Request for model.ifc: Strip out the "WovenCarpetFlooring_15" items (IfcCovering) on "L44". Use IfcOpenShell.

First a look at what the model holds.

```python
import ifcopenshell
import ifcopenshell.util.element

model = ifcopenshell.open("model.ifc")
print(model.schema)
storey = next(s for s in model.by_type("IfcBuildingStorey") if s.Name == "L44")
coverings = [e for e in ifcopenshell.util.element.get_decomposition(storey) if e.is_a("IfcCovering")]
seen = {}
for e in coverings:
    element_type = ifcopenshell.util.element.get_type(e)
    name = element_type.Name if element_type not in (None, e) else None
    seen[name] = seen.get(name, 0) + 1
for name, count in sorted(seen.items(), key=str):
    print(count, "x", name)
```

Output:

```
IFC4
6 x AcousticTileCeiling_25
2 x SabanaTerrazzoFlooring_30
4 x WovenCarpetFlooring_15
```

```python
import ifcopenshell
import ifcopenshell.api.root
import ifcopenshell.util.element

model = ifcopenshell.open("model.ifc")

storey = next(s for s in model.by_type("IfcBuildingStorey") if s.Name == "L44")
coverings = [e for e in ifcopenshell.util.element.get_decomposition(storey) if e.is_a("IfcCovering")]
targets = [e for e in coverings if (t := ifcopenshell.util.element.get_type(e)) not in (None, e) and t.Name == "WovenCarpetFlooring_15"]

for e in targets:
    ifcopenshell.api.root.remove_product(model, product=e)
print(len(targets), "removed")

model.write("model_edited.ifc")
```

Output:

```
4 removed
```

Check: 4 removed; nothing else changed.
